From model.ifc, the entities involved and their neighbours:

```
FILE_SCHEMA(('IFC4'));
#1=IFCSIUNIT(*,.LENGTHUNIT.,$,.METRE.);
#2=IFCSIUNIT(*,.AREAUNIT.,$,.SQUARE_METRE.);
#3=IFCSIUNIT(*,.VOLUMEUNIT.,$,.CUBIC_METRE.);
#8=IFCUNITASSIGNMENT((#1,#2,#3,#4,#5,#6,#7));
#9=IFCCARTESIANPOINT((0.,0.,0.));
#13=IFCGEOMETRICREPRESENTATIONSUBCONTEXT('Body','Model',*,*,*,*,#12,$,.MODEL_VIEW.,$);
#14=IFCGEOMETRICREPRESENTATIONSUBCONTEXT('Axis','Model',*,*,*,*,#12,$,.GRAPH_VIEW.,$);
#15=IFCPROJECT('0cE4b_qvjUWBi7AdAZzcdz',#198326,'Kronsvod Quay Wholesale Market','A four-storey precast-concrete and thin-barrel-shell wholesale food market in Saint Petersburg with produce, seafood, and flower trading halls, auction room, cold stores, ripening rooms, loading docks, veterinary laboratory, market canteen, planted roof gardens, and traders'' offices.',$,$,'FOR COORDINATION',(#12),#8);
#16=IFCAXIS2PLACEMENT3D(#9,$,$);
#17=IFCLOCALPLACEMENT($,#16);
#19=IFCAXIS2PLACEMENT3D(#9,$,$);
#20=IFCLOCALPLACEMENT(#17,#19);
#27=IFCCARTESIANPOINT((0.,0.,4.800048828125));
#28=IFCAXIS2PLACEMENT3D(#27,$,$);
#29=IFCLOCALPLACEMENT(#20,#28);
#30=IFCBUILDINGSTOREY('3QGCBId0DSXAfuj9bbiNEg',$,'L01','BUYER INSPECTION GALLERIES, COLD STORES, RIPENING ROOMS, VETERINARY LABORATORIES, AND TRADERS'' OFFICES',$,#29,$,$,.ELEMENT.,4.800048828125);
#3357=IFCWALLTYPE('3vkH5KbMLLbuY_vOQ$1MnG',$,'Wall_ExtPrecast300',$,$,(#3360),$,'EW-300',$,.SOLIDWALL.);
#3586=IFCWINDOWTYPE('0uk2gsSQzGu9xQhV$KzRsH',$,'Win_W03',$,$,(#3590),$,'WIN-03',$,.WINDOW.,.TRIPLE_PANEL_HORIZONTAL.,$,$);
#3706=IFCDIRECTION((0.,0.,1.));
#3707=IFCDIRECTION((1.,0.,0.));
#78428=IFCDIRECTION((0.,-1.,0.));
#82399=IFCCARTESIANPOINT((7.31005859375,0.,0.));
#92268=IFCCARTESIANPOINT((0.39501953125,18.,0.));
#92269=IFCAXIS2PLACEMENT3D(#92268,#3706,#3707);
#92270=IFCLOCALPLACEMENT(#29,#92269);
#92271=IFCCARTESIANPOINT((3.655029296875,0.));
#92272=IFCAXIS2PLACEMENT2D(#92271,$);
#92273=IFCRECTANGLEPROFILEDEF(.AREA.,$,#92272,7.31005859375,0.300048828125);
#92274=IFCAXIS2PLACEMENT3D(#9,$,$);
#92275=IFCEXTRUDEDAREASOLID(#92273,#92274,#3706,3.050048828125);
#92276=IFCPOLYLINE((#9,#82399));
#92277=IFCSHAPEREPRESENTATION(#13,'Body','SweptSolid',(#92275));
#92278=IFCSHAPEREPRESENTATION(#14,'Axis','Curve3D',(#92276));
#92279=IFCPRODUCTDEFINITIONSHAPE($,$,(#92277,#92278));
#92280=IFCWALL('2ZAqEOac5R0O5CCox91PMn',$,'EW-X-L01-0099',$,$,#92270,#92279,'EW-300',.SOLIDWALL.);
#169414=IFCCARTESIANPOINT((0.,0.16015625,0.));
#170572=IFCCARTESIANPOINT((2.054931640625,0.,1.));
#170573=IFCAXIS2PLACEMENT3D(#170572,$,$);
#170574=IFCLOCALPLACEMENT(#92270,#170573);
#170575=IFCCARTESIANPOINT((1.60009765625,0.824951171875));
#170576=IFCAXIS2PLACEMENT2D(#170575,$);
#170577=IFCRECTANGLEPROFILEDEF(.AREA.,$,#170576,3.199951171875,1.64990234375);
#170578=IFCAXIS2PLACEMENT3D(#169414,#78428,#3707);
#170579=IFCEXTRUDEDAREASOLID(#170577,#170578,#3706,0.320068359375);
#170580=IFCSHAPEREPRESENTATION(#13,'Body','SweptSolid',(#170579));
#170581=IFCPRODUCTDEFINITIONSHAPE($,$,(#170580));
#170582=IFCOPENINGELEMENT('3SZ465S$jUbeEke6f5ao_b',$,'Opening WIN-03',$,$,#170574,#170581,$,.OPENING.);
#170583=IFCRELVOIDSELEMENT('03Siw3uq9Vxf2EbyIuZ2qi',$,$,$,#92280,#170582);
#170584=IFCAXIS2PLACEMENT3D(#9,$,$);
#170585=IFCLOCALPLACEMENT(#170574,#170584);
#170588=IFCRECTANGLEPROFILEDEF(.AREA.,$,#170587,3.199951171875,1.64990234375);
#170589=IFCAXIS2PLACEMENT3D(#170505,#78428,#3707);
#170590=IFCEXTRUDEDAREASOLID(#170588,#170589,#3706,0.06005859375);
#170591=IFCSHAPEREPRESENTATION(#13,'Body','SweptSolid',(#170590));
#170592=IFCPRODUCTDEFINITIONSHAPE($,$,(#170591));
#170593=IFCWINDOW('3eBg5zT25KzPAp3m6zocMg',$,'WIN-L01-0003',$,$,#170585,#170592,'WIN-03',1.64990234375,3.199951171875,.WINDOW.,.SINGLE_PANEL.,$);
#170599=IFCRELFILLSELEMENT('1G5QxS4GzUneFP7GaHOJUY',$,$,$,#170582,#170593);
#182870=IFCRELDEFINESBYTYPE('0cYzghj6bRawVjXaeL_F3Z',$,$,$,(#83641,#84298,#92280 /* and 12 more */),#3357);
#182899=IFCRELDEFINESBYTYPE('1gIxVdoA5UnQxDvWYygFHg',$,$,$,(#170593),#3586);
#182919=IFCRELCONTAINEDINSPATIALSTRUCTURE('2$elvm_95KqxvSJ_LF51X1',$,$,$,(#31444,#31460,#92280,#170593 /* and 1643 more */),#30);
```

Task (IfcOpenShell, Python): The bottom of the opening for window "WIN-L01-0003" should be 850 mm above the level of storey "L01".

```python
import numpy as np
import ifcopenshell
import ifcopenshell.api.geometry
import ifcopenshell.geom
import ifcopenshell.util.element
import ifcopenshell.util.placement
import ifcopenshell.util.shape
import ifcopenshell.util.unit

model = ifcopenshell.open("model.ifc")
unit_scale = ifcopenshell.util.unit.calculate_unit_scale(model)

window = model.by_guid("3eBg5zT25KzPAp3m6zocMg")
opening = window.FillsVoids[0].RelatingOpeningElement
storey = ifcopenshell.util.element.get_container(window, ifc_class="IfcBuildingStorey")
level = ifcopenshell.util.placement.get_local_placement(storey.ObjectPlacement)[2, 3]

# The opening's origin need not be at the sill, so measure its lowest point.
shape = ifcopenshell.geom.create_shape(ifcopenshell.geom.settings(), opening)
bottom = ifcopenshell.util.shape.get_shape_bottom_elevation(shape, shape.geometry) / unit_scale
dz = level + 0.85 / unit_scale - bottom

shift = np.array([0.0, 0.0, dz])
# The window is placed relative to its opening, so it follows when the opening moves.
matrix = ifcopenshell.util.placement.get_local_placement(opening.ObjectPlacement)
matrix[:3, 3] += shift
ifcopenshell.api.geometry.edit_object_placement(
    model, product=opening, matrix=matrix, is_si=False, should_transform_children=True
)

print(f"moved by {dz * unit_scale:+.3f} m")

model.write("model_v2.ifc")
```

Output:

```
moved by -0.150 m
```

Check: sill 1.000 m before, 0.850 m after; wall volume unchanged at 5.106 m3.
